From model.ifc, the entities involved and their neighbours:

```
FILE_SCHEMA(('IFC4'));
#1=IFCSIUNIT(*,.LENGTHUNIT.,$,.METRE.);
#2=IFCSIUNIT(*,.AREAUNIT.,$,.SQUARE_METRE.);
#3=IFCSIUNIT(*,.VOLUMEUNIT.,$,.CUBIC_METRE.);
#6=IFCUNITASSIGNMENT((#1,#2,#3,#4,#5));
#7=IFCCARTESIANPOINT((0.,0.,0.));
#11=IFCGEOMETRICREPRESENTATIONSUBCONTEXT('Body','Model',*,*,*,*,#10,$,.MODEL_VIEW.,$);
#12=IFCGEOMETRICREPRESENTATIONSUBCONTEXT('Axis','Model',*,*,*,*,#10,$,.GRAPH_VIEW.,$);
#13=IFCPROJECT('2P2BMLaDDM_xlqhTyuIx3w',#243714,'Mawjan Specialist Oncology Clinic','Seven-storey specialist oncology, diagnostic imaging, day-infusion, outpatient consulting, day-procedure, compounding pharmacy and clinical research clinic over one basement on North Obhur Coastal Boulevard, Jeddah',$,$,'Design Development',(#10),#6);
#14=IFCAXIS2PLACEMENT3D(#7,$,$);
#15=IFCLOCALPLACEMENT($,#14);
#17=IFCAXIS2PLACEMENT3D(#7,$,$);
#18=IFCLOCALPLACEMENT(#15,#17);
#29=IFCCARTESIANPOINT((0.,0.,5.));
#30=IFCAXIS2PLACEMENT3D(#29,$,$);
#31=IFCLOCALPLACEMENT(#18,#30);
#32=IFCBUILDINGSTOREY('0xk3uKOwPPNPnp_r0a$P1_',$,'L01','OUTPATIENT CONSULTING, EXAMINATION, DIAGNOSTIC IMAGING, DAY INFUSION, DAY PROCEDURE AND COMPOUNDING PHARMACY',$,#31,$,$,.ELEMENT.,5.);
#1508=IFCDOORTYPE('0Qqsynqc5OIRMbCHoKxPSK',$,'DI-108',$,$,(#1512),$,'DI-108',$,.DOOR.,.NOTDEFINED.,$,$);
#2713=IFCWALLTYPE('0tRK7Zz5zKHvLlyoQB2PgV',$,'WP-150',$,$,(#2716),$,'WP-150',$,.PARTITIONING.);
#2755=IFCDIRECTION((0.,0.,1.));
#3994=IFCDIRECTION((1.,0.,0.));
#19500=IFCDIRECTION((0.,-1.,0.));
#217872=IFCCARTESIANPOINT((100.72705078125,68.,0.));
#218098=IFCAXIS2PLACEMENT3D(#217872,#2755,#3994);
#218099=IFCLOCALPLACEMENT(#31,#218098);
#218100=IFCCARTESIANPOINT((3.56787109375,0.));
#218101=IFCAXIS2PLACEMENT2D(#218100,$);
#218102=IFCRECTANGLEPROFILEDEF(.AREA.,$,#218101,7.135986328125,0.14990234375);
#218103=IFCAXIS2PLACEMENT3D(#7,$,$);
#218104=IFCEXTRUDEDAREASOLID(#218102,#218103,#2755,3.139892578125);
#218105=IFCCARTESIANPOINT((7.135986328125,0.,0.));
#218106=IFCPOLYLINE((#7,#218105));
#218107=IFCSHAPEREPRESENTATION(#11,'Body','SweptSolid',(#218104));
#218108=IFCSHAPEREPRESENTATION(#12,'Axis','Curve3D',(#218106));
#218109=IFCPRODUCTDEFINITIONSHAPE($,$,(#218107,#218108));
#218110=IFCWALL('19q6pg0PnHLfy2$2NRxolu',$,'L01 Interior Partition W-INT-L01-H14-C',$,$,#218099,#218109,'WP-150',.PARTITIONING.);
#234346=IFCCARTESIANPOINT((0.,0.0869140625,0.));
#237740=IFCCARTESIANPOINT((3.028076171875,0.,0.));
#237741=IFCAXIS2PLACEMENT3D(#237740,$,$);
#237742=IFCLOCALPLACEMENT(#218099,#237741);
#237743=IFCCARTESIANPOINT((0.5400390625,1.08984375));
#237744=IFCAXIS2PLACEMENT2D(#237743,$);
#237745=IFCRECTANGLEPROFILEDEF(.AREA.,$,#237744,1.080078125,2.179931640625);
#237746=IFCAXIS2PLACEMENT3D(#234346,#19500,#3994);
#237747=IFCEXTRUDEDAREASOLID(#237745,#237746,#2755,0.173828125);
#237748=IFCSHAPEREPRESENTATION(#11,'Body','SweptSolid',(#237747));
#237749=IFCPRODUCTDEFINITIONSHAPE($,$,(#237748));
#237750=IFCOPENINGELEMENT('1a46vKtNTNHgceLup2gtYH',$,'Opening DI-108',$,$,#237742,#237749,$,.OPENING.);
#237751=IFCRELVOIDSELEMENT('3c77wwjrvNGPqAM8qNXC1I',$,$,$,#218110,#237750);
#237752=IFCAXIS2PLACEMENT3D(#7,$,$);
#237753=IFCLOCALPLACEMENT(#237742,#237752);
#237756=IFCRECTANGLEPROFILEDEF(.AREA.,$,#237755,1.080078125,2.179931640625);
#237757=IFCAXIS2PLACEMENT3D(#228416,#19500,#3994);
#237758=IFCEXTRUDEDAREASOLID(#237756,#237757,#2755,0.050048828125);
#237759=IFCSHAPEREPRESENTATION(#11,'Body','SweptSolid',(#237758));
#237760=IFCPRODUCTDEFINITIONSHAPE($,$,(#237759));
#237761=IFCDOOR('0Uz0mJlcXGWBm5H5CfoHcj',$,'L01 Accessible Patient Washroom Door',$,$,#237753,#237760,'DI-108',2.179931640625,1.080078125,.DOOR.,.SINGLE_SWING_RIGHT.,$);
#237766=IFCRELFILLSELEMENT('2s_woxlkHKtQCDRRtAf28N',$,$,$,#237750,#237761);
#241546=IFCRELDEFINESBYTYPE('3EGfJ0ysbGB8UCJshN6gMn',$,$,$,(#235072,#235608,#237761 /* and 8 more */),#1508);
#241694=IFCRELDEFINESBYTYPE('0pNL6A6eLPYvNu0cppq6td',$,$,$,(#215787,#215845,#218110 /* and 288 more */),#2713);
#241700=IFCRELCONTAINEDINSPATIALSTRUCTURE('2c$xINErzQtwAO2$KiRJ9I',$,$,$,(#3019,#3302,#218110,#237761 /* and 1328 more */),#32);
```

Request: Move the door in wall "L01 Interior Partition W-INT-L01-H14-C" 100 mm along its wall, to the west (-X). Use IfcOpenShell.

```python
import ifcopenshell
import ifcopenshell.api.geometry
import ifcopenshell.util.placement
import ifcopenshell.util.unit

model = ifcopenshell.open("model.ifc")
unit_scale = ifcopenshell.util.unit.calculate_unit_scale(model)

door = model.by_guid("0Uz0mJlcXGWBm5H5CfoHcj")
opening = door.FillsVoids[0].RelatingOpeningElement
wall = opening.VoidsElements[0].RelatingBuildingElement

wall_matrix = ifcopenshell.util.placement.get_local_placement(wall.ObjectPlacement)
shift = wall_matrix[:3, 0] * -0.1 / unit_scale
before = ifcopenshell.util.placement.get_local_placement(door.ObjectPlacement)[:3, 3].copy()

# The door is placed relative to its opening, so it follows when the opening moves.
matrix = ifcopenshell.util.placement.get_local_placement(opening.ObjectPlacement)
matrix[:3, 3] += shift
ifcopenshell.api.geometry.edit_object_placement(
    model, product=opening, matrix=matrix, is_si=False, should_transform_children=True
)

after = ifcopenshell.util.placement.get_local_placement(door.ObjectPlacement)[:3, 3]
print("door moved by", (after - before).round(3) + 0.0)

model.write("model_v2.ifc")
```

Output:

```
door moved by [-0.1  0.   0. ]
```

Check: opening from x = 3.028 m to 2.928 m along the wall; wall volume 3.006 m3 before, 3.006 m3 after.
